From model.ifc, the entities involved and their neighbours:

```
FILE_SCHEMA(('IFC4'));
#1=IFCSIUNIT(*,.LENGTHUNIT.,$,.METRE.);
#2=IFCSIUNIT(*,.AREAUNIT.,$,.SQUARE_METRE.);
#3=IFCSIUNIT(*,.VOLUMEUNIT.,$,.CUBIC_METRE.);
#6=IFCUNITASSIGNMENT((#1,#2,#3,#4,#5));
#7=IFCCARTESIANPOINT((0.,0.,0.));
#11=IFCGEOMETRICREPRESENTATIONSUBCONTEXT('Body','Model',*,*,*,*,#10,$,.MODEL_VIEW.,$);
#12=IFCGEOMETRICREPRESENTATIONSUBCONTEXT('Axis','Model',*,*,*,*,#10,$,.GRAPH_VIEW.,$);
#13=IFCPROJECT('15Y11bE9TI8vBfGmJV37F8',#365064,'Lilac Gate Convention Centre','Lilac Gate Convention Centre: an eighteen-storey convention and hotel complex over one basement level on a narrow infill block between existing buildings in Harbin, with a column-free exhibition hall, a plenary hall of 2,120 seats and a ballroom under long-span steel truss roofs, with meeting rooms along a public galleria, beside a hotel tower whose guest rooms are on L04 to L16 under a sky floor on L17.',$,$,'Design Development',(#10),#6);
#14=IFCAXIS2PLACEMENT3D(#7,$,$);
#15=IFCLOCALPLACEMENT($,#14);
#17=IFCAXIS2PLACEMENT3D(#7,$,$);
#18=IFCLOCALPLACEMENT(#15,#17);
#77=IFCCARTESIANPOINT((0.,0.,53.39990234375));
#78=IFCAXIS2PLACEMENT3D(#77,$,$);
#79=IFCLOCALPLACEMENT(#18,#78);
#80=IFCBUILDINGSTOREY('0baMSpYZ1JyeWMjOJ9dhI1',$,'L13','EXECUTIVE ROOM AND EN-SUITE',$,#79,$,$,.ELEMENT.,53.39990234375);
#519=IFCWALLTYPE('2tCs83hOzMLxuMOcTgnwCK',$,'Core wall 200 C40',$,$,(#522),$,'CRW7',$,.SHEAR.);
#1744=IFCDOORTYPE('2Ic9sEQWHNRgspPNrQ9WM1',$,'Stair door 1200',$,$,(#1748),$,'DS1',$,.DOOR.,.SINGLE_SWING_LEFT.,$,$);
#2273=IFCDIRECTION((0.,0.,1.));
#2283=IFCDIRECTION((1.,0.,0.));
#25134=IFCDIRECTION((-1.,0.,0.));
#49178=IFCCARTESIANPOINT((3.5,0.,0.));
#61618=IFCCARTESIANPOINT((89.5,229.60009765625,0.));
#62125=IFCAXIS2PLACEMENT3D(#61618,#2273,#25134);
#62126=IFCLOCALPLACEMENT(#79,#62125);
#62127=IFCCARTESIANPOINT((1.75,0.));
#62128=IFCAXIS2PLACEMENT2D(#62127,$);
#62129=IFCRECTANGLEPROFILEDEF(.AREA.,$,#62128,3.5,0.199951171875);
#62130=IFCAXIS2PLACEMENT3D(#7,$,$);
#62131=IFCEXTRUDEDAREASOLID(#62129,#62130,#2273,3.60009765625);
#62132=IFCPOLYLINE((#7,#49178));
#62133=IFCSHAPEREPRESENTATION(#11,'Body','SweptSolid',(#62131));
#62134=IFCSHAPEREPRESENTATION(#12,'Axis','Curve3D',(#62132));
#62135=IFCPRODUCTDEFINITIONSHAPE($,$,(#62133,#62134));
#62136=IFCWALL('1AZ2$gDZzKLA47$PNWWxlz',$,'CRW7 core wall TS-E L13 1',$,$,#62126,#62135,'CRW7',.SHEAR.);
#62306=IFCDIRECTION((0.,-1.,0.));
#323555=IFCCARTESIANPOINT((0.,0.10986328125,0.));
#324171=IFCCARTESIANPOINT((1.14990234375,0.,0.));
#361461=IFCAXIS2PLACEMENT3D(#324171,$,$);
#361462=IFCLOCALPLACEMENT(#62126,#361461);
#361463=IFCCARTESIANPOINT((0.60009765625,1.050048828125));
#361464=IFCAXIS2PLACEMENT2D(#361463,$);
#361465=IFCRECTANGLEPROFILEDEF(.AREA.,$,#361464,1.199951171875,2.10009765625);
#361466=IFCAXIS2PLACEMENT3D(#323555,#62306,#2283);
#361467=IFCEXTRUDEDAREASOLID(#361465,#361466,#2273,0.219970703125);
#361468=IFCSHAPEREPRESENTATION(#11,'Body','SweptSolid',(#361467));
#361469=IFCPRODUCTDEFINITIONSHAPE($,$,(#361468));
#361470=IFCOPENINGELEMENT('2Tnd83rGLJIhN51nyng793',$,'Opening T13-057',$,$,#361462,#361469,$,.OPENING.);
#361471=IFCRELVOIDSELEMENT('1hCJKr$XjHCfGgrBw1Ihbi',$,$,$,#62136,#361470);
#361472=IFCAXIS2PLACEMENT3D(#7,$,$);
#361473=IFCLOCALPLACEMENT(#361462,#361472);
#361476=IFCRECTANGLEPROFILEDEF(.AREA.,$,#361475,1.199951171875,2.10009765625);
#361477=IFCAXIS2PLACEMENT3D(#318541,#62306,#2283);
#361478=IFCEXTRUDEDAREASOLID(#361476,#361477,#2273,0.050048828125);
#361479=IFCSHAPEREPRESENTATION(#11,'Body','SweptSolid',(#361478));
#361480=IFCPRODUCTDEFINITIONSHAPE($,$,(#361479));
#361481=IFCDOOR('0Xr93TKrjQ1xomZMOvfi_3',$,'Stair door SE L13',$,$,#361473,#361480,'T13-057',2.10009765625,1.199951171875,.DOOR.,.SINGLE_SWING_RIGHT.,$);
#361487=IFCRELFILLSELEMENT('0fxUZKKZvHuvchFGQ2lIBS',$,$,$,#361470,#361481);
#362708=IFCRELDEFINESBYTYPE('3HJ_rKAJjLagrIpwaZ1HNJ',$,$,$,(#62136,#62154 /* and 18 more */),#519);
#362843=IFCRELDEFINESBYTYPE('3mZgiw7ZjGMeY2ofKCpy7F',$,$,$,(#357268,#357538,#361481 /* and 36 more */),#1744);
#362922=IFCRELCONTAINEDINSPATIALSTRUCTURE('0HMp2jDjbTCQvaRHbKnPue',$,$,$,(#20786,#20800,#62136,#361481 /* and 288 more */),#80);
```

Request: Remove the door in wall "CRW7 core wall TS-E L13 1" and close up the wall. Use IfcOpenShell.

```python
import ifcopenshell
import ifcopenshell.api.feature
import ifcopenshell.api.root
import ifcopenshell.geom
import ifcopenshell.util.shape

model = ifcopenshell.open("model.ifc")
settings = ifcopenshell.geom.settings()


def volume(element):
    """Net volume in cubic metres, openings subtracted."""
    shape = ifcopenshell.geom.create_shape(settings, element)
    return ifcopenshell.util.shape.get_volume(shape.geometry)


door = model.by_id(361481)
opening = door.FillsVoids[0].RelatingOpeningElement
wall = opening.VoidsElements[0].RelatingBuildingElement
before = volume(wall)

ifcopenshell.api.root.remove_product(model, product=door)
ifcopenshell.api.feature.remove_feature(model, feature=opening)

after = volume(wall)

print(f"wall volume {before:.3f} -> {after:.3f} m3")

model.write("model-out.ifc")
```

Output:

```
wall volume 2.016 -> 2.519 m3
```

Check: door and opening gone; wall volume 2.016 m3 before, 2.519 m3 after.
